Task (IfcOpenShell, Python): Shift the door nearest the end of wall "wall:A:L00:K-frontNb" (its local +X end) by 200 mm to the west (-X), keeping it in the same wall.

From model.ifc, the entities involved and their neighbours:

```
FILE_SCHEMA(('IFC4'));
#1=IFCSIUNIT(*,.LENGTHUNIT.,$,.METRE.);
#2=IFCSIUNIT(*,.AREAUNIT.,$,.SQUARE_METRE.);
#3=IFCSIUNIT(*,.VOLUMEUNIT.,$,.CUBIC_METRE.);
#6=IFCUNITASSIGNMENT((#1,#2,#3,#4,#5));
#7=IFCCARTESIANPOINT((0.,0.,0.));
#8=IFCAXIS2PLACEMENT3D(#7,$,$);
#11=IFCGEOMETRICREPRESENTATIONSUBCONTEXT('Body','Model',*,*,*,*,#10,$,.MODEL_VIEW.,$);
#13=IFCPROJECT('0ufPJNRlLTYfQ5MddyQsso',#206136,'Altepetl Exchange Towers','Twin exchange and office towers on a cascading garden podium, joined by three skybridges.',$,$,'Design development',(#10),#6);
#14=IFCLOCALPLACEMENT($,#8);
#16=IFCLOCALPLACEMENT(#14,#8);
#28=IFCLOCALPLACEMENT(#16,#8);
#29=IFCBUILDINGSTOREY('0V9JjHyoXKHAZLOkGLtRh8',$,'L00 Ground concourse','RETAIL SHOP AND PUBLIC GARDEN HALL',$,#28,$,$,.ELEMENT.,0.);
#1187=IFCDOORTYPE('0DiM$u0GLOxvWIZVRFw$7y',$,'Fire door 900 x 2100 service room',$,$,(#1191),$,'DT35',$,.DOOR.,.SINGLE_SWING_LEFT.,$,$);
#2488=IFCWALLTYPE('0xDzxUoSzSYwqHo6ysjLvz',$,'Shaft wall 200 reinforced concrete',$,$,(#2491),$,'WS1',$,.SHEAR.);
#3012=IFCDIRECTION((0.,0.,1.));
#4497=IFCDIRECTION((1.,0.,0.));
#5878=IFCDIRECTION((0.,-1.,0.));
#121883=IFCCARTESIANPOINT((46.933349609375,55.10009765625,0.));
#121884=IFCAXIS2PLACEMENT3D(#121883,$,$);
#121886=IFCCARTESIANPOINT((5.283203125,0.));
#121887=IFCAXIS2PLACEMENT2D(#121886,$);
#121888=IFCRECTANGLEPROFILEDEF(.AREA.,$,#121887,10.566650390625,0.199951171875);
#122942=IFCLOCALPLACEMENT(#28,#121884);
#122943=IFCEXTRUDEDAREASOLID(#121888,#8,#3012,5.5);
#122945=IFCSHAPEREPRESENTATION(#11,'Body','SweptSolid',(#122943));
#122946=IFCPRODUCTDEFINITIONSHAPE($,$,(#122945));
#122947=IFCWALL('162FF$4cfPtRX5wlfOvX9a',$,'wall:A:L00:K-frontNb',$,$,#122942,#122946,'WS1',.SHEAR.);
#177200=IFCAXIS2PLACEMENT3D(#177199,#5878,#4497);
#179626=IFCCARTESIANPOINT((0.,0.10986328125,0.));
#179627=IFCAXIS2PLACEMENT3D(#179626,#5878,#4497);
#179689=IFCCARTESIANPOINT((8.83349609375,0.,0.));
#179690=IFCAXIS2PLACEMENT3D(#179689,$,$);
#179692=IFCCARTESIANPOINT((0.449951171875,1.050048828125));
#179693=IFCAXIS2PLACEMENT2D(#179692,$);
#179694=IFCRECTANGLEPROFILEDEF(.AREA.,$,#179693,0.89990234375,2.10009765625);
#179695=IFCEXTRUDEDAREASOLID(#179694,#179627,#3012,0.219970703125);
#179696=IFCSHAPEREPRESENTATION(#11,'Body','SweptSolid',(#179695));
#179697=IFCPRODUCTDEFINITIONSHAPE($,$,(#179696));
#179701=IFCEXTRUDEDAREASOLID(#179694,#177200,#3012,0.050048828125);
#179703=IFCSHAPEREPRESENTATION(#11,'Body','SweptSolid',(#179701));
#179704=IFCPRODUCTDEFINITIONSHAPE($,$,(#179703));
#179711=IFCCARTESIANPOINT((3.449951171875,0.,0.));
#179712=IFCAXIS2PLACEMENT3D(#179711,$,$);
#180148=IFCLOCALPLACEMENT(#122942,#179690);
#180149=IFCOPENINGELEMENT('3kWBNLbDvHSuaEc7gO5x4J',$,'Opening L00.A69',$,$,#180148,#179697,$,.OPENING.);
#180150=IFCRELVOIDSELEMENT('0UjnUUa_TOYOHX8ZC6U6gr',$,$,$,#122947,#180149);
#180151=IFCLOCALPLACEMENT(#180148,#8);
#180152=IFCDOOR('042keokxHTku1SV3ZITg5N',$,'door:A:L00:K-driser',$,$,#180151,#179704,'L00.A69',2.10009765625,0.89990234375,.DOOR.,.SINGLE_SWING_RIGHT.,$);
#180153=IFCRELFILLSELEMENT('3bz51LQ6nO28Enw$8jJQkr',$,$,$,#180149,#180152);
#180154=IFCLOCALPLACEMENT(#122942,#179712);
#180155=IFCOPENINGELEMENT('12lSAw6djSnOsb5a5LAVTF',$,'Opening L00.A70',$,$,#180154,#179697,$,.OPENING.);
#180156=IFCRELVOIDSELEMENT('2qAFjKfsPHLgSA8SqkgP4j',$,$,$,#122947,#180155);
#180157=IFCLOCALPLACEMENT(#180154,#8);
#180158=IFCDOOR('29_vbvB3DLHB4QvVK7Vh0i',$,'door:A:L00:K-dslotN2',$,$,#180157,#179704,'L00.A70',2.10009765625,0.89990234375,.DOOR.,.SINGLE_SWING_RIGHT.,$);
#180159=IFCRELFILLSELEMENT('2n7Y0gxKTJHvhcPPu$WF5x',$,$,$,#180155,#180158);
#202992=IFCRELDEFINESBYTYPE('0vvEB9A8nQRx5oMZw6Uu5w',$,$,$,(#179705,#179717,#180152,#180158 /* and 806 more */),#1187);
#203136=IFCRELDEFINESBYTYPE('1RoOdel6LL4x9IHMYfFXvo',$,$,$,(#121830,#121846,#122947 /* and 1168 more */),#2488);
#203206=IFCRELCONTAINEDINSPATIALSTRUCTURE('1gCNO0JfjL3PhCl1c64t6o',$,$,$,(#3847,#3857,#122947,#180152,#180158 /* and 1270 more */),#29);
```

```python
import ifcopenshell
import ifcopenshell.api.geometry
import ifcopenshell.util.placement

model = ifcopenshell.open("model.ifc")

door = model.by_guid("042keokxHTku1SV3ZITg5N")
opening = door.FillsVoids[0].RelatingOpeningElement
wall = opening.VoidsElements[0].RelatingBuildingElement

wall_matrix = ifcopenshell.util.placement.get_local_placement(wall.ObjectPlacement)
shift = wall_matrix[:3, 0] * -0.2
before = ifcopenshell.util.placement.get_local_placement(door.ObjectPlacement)[:3, 3].copy()

# The door is placed relative to its opening, so it follows when the opening moves.
matrix = ifcopenshell.util.placement.get_local_placement(opening.ObjectPlacement)
matrix[:3, 3] += shift
ifcopenshell.api.geometry.edit_object_placement(
    model, product=opening, matrix=matrix, is_si=False, should_transform_children=True
)

after = ifcopenshell.util.placement.get_local_placement(door.ObjectPlacement)[:3, 3]
print("door moved by", (after - before).round(3) + 0.0)

model.write("model-out.ifc")
```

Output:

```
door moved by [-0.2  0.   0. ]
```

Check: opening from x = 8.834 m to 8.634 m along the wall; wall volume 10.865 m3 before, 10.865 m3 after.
